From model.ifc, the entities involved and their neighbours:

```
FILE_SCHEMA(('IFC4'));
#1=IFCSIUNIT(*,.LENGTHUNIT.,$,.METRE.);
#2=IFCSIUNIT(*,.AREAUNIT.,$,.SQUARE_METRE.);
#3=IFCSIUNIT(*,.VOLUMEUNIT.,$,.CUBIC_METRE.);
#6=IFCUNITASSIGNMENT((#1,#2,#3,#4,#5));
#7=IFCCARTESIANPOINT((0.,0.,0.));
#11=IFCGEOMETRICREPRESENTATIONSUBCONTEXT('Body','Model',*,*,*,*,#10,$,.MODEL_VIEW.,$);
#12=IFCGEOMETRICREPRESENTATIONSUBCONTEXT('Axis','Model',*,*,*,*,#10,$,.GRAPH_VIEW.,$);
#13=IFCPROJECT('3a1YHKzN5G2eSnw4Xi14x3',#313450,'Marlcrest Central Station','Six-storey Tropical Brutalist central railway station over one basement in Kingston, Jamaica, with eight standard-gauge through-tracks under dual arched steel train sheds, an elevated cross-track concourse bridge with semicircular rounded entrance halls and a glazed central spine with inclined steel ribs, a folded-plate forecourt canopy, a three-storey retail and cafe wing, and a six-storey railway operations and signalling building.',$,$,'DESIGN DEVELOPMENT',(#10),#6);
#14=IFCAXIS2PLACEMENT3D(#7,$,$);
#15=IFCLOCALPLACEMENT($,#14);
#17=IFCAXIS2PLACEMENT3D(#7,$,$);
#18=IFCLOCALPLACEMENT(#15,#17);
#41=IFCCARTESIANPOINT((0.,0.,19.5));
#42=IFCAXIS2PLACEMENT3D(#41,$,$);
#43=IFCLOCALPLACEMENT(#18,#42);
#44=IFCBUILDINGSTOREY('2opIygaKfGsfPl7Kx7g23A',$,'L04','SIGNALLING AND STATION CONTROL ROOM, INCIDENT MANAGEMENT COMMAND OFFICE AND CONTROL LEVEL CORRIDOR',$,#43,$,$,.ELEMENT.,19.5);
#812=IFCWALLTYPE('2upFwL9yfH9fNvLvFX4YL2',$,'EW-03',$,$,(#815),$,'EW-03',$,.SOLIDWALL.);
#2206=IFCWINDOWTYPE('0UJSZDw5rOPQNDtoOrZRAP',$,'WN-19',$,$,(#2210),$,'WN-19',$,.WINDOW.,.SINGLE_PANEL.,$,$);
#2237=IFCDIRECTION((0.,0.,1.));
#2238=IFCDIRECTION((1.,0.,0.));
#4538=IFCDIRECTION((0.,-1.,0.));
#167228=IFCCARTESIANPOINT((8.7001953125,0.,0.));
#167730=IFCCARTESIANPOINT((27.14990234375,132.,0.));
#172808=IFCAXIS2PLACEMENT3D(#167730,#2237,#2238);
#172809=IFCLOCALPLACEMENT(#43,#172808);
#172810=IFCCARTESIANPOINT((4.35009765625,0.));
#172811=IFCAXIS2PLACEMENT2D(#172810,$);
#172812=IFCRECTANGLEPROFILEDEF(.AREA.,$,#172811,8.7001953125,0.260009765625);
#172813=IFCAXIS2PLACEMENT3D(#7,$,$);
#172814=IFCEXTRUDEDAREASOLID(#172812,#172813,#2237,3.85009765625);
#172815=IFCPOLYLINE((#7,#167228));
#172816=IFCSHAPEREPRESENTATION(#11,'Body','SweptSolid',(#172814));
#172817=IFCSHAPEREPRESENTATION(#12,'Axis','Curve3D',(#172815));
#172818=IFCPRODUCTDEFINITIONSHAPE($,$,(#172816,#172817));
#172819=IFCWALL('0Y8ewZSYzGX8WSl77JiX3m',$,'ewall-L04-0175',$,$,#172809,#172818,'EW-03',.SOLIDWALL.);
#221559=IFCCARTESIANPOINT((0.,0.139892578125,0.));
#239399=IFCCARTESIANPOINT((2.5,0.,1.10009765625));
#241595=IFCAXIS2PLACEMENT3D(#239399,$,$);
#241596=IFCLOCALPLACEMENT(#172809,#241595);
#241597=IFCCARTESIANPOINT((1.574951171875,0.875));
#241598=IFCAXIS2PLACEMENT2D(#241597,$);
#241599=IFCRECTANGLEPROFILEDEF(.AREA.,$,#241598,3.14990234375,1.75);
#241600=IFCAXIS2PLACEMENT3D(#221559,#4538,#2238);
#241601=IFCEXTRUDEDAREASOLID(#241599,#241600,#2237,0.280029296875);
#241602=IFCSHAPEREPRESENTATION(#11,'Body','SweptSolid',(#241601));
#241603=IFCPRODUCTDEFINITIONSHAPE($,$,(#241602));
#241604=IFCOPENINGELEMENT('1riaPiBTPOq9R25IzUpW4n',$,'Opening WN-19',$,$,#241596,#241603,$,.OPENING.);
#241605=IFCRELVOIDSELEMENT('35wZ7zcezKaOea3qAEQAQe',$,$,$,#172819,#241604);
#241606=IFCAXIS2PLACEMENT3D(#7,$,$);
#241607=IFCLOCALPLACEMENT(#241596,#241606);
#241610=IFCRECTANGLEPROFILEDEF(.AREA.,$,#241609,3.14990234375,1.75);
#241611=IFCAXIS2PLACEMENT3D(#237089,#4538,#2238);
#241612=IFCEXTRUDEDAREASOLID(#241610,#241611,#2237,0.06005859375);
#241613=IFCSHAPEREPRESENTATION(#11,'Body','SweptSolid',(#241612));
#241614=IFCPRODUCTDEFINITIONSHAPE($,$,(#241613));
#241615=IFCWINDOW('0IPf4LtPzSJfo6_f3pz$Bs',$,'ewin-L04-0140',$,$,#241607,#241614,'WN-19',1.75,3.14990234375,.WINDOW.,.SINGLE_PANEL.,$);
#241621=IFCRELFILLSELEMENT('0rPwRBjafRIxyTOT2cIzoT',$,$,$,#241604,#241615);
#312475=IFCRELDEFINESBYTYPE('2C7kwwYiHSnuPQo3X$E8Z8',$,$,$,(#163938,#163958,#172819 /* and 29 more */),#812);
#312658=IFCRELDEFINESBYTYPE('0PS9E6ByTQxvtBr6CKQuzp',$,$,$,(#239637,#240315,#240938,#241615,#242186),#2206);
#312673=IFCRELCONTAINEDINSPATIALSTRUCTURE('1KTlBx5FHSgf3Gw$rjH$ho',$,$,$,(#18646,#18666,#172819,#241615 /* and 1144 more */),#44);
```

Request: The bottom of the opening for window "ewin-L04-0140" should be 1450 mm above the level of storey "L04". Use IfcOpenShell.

```python
import numpy as np
import ifcopenshell
import ifcopenshell.api.geometry
import ifcopenshell.geom
import ifcopenshell.util.element
import ifcopenshell.util.placement
import ifcopenshell.util.shape
import ifcopenshell.util.unit

model = ifcopenshell.open("model.ifc")
unit_scale = ifcopenshell.util.unit.calculate_unit_scale(model)

window = model.by_id(241615)
opening = window.FillsVoids[0].RelatingOpeningElement
storey = ifcopenshell.util.element.get_container(window, ifc_class="IfcBuildingStorey")
level = ifcopenshell.util.placement.get_local_placement(storey.ObjectPlacement)[2, 3]

# The opening's origin need not be at the sill, so measure its lowest point.
shape = ifcopenshell.geom.create_shape(ifcopenshell.geom.settings(), opening)
bottom = ifcopenshell.util.shape.get_shape_bottom_elevation(shape, shape.geometry) / unit_scale
dz = level + 1.45 / unit_scale - bottom

shift = np.array([0.0, 0.0, dz])
# The window is placed relative to its opening, so it follows when the opening moves.
matrix = ifcopenshell.util.placement.get_local_placement(opening.ObjectPlacement)
matrix[:3, 3] += shift
ifcopenshell.api.geometry.edit_object_placement(
    model, product=opening, matrix=matrix, is_si=False, should_transform_children=True
)

print(f"moved by {dz * unit_scale:+.3f} m")

model.write("model_updated.ifc")
```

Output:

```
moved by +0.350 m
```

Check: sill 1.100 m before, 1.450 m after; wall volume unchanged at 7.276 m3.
